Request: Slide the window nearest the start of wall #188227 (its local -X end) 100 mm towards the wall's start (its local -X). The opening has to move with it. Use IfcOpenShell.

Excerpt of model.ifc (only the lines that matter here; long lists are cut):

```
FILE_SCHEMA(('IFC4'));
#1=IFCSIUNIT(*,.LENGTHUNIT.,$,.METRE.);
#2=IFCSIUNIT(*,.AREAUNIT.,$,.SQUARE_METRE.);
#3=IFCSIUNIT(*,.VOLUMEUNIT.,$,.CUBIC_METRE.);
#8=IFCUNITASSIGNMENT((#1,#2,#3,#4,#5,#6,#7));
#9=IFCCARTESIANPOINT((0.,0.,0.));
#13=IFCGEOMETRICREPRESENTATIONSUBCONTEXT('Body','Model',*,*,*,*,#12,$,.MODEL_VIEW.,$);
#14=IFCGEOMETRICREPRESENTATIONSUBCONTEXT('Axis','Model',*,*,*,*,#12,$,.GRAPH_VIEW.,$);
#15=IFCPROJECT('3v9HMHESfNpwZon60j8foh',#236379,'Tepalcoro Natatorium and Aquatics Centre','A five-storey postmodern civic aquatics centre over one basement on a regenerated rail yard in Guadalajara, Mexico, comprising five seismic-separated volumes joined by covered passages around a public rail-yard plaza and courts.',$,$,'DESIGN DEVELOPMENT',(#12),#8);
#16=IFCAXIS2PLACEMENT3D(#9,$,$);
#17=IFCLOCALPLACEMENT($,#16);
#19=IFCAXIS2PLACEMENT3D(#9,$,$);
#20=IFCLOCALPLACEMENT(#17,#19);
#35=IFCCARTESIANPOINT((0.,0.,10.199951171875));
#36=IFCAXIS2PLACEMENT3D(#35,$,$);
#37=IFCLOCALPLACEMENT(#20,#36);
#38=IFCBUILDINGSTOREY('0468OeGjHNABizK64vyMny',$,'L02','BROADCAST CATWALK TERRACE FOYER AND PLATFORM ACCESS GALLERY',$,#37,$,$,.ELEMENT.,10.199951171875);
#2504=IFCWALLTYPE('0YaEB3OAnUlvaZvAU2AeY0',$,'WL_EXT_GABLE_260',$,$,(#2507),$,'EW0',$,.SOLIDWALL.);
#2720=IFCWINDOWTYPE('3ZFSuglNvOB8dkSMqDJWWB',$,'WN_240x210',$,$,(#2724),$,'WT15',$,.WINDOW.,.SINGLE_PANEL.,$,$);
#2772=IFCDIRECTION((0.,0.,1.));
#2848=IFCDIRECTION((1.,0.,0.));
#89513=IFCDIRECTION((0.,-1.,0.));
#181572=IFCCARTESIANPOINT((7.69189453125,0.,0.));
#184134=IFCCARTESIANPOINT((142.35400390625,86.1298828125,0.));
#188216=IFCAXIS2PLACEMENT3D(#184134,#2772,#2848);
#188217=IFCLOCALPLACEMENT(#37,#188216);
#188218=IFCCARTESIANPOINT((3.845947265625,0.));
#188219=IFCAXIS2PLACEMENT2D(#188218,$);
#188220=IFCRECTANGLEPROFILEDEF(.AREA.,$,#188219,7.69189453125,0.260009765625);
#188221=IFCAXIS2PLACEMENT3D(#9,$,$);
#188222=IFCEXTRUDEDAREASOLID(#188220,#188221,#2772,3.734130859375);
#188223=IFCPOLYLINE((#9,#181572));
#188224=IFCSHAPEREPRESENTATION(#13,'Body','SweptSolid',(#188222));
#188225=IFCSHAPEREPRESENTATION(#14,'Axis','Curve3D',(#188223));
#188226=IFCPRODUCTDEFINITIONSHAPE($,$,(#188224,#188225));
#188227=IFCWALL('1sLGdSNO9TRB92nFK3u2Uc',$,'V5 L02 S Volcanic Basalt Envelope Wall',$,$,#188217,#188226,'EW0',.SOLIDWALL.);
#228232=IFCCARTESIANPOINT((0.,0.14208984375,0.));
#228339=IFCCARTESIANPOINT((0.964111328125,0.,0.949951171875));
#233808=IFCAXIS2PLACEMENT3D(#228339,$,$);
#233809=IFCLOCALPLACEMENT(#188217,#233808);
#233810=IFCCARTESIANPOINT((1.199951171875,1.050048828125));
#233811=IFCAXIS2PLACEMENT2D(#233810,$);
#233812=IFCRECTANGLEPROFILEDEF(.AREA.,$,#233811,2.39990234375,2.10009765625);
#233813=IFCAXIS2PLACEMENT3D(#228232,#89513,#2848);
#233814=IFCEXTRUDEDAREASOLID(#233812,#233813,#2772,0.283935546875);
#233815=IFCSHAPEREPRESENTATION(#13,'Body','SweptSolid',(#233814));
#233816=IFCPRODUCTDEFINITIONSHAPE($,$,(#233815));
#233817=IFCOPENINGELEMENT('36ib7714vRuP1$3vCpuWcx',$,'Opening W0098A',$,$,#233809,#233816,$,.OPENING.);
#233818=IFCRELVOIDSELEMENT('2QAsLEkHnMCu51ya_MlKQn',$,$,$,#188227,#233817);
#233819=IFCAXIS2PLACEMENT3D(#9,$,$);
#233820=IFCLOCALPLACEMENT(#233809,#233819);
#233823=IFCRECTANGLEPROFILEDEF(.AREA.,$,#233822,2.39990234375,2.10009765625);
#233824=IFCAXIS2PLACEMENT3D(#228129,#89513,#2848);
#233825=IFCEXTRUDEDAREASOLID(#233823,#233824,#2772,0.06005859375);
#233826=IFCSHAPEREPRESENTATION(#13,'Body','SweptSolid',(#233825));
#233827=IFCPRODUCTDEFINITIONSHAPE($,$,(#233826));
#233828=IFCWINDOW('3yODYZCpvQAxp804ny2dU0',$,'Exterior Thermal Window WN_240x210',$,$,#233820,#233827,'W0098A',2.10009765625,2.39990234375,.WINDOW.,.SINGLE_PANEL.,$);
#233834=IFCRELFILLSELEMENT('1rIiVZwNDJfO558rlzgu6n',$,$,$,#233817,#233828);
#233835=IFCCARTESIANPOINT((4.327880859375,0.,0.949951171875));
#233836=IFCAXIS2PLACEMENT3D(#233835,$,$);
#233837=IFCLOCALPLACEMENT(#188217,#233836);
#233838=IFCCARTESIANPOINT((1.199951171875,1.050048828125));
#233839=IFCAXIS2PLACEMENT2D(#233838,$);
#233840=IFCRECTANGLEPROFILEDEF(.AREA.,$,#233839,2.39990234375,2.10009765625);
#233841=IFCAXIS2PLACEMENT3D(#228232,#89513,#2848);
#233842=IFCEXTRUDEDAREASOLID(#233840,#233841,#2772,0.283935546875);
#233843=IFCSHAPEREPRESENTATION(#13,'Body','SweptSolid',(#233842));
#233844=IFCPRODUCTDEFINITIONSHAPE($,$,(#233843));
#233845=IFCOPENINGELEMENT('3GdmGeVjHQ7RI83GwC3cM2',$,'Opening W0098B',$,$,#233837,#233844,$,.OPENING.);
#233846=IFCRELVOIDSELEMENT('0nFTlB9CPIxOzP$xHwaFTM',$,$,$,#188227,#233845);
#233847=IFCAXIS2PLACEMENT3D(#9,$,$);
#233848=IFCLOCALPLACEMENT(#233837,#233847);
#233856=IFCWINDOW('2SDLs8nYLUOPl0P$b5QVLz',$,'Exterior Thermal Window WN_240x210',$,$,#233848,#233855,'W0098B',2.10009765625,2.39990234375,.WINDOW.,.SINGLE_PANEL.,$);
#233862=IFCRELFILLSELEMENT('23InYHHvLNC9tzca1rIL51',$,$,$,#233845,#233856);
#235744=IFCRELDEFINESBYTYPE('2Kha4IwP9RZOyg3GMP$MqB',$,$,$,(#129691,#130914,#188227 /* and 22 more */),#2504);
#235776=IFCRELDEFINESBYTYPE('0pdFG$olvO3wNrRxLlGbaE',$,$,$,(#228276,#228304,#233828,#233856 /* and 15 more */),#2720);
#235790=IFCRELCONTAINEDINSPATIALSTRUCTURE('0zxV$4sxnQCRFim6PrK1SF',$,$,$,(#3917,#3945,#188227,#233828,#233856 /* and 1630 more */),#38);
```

```python
import ifcopenshell
import ifcopenshell.api.geometry
import ifcopenshell.util.placement

model = ifcopenshell.open("model.ifc")

window = model.by_guid("3yODYZCpvQAxp804ny2dU0")
opening = window.FillsVoids[0].RelatingOpeningElement
wall = opening.VoidsElements[0].RelatingBuildingElement

wall_matrix = ifcopenshell.util.placement.get_local_placement(wall.ObjectPlacement)
shift = wall_matrix[:3, 0] * -0.1
before = ifcopenshell.util.placement.get_local_placement(window.ObjectPlacement)[:3, 3].copy()

# The window is placed relative to its opening, so it follows when the opening moves.
matrix = ifcopenshell.util.placement.get_local_placement(opening.ObjectPlacement)
matrix[:3, 3] += shift
ifcopenshell.api.geometry.edit_object_placement(
    model, product=opening, matrix=matrix, is_si=False, should_transform_children=True
)

after = ifcopenshell.util.placement.get_local_placement(window.ObjectPlacement)[:3, 3]
print("window moved by", (after - before).round(3) + 0.0)

model.write("model_edited.ifc")
```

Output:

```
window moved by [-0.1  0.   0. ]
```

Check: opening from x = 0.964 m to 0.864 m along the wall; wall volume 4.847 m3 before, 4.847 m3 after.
